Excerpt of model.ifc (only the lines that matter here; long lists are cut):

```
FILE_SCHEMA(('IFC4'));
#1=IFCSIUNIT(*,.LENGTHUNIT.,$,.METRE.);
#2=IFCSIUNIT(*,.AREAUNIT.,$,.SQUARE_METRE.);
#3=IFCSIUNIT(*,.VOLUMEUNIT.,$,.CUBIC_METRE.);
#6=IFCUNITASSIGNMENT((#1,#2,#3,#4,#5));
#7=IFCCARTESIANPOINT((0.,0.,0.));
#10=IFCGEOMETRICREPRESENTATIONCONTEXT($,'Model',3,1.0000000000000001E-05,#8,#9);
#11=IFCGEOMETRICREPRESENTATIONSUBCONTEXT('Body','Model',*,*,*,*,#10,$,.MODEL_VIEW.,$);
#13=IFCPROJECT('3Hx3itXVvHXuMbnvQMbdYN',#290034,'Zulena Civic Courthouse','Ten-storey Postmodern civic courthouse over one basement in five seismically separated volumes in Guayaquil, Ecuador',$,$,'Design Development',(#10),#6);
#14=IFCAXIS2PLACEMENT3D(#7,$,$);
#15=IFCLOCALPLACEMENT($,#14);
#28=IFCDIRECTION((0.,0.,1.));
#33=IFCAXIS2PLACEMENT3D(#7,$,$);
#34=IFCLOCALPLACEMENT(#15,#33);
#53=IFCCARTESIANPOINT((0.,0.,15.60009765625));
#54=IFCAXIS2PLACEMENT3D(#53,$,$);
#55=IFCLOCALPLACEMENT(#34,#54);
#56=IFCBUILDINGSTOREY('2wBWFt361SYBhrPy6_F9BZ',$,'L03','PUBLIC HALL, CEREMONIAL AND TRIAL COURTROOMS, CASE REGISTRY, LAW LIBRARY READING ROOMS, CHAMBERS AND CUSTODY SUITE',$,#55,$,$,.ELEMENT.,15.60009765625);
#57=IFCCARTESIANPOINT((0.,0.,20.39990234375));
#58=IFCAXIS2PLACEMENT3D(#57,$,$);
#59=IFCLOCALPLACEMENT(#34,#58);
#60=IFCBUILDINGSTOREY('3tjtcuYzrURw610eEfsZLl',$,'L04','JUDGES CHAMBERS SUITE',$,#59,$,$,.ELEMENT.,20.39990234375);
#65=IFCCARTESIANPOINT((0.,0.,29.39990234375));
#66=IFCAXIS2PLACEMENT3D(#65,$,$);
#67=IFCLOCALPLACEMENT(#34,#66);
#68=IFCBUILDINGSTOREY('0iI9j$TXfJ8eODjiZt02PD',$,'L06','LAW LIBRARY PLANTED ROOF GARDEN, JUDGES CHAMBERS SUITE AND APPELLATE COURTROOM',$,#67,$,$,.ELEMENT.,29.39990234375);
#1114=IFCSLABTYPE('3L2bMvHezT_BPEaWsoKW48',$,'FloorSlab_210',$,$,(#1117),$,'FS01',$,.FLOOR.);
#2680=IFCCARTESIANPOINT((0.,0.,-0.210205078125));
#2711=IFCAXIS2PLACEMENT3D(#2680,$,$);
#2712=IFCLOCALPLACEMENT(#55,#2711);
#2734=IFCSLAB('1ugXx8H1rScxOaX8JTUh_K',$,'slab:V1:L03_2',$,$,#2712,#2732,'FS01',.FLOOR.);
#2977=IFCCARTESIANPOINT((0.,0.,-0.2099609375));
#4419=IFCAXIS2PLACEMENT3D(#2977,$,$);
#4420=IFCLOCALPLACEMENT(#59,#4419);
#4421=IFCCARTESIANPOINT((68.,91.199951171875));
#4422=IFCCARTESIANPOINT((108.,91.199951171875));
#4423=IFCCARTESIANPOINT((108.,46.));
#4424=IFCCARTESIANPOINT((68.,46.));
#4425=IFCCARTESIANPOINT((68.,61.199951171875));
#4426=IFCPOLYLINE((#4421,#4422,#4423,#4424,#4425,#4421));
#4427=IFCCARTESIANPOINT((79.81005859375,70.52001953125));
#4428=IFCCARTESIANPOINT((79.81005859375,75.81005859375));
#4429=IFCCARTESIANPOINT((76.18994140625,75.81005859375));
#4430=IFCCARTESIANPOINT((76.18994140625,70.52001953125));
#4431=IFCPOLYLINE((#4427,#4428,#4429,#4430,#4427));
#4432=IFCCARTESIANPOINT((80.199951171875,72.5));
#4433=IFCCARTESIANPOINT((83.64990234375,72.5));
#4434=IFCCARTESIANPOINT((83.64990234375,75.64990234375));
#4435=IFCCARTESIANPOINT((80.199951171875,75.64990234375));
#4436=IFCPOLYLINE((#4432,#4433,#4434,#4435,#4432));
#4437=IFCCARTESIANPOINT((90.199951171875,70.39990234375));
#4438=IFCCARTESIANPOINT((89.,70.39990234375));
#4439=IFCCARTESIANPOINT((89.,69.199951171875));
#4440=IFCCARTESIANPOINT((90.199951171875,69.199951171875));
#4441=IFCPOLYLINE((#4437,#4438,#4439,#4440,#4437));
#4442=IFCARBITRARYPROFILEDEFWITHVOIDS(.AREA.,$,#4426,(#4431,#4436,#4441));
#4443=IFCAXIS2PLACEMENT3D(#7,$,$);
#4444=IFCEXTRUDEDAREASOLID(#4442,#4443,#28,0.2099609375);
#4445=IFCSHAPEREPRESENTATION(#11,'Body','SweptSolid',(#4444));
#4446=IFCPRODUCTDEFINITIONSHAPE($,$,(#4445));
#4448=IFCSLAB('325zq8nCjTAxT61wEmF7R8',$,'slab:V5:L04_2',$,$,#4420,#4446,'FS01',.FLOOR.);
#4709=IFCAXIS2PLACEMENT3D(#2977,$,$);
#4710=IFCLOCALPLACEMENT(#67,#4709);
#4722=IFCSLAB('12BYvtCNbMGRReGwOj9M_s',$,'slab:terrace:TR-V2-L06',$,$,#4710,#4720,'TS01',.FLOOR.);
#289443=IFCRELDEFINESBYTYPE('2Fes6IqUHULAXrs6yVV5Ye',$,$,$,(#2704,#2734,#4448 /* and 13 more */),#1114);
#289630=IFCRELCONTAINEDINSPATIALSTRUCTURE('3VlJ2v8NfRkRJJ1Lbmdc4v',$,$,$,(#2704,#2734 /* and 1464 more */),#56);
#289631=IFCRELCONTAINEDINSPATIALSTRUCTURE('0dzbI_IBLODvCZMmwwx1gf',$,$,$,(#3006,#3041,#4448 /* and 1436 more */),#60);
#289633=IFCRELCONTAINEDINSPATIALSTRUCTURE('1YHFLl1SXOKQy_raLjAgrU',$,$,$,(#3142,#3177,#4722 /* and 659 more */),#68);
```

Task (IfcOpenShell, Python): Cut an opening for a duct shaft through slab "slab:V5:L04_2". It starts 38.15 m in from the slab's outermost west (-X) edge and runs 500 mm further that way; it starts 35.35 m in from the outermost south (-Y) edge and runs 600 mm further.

```python
import numpy as np
import ifcopenshell
import ifcopenshell.api.feature
import ifcopenshell.api.geometry
import ifcopenshell.api.root
import ifcopenshell.geom
import ifcopenshell.util.placement
import ifcopenshell.util.representation
import ifcopenshell.util.shape
import ifcopenshell.util.unit

model = ifcopenshell.open("model.ifc")
unit_scale = ifcopenshell.util.unit.calculate_unit_scale(model)
settings = ifcopenshell.geom.settings()


def volume(element):
    """Net volume in cubic metres, openings subtracted."""
    shape = ifcopenshell.geom.create_shape(settings, element)
    return ifcopenshell.util.shape.get_volume(shape.geometry)


slab = model.by_guid("325zq8nCjTAxT61wEmF7R8")
before = volume(slab)

# Extent in the slab's own axes, in metres. The edges named are its -X and -Y sides.
slab_shape = ifcopenshell.geom.create_shape(settings, slab)
vertices = ifcopenshell.util.shape.get_vertices(slab_shape.geometry)
x_min, y_min, bottom = vertices.min(axis=0)
top = vertices[:, 2].max()

opening = ifcopenshell.api.root.create_entity(model, ifc_class="IfcOpeningElement", name="Duct shaft opening", predefined_type="OPENING")
context = ifcopenshell.util.representation.get_context(model, "Model", "Body", "MODEL_VIEW")
width, depth = 0.5, 0.6
outline = [(0.0, 0.0), (width, 0.0), (width, depth), (0.0, depth), (0.0, 0.0)]
# Overshoot both faces by 50 mm so the cut is clean.
shape = ifcopenshell.api.geometry.add_slab_representation(
    model, context=context, depth=top - bottom + 0.1, polyline=outline
)
ifcopenshell.api.geometry.assign_representation(model, product=opening, representation=shape)

matrix = ifcopenshell.util.placement.get_local_placement(slab.ObjectPlacement)
matrix[:, 3] = matrix @ np.append(np.array([x_min + 38.15, y_min + 35.35, bottom - 0.05]) / unit_scale, 1.0)
ifcopenshell.api.geometry.edit_object_placement(model, product=opening, matrix=matrix, is_si=False)
ifcopenshell.api.feature.add_feature(model, feature=opening, element=slab)

after = volume(slab)

print(f"slab volume {before:.3f} -> {after:.3f} m3")

model.write("model_v2.ifc")
```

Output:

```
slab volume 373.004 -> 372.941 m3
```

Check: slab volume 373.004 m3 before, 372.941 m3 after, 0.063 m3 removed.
